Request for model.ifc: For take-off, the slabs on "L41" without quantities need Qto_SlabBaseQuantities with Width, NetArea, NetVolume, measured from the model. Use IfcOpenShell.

First a look at what the model holds.

```python
import ifcopenshell
import ifcopenshell.util.element
import ifcopenshell.util.unit

model = ifcopenshell.open("model.ifc")
print(model.schema)
for unit_type in ("LENGTHUNIT", "AREAUNIT", "VOLUMEUNIT"):
    print(unit_type, ifcopenshell.util.unit.calculate_unit_scale(model, unit_type))
storey = next(s for s in model.by_type("IfcBuildingStorey") if s.Name == "L41")
slabs = [e for e in ifcopenshell.util.element.get_decomposition(storey) if e.is_a("IfcSlab")]
for e in sorted(slabs, key=lambda e: e.id()):
    print(e.id(), e.is_a(), e.Name, list(ifcopenshell.util.element.get_psets(e, qtos_only=True)), sep=" | ")
```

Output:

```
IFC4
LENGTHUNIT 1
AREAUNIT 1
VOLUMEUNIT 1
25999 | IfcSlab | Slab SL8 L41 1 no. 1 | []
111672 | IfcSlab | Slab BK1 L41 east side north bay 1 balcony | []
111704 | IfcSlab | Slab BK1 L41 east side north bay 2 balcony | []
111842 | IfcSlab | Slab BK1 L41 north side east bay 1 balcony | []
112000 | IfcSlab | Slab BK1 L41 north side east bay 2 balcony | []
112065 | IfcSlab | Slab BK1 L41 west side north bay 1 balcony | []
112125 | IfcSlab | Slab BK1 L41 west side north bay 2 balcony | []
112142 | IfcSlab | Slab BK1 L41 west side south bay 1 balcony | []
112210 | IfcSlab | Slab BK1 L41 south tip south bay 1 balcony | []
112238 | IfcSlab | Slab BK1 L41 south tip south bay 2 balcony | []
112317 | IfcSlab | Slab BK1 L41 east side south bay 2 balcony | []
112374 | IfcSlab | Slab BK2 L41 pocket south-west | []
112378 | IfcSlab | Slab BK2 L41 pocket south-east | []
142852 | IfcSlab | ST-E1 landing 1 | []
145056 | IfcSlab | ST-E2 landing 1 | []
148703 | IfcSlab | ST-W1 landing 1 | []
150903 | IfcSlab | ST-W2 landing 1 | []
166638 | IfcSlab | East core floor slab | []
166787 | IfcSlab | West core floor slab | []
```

```python
import ifcopenshell
import ifcopenshell.api.pset
import ifcopenshell.geom
import ifcopenshell.util.element
import ifcopenshell.util.shape
import ifcopenshell.util.unit

model = ifcopenshell.open("model.ifc")
unit_scale = ifcopenshell.util.unit.calculate_unit_scale(model)
area_scale = ifcopenshell.util.unit.calculate_unit_scale(model, "AREAUNIT")
volume_scale = ifcopenshell.util.unit.calculate_unit_scale(model, "VOLUMEUNIT")
settings = ifcopenshell.geom.settings()

storey = next(s for s in model.by_type("IfcBuildingStorey") if s.Name == "L41")
slabs = [e for e in ifcopenshell.util.element.get_decomposition(storey) if e.is_a("IfcSlab")]

for e in sorted(slabs, key=lambda e: e.id()):
    if ifcopenshell.util.element.get_psets(e, qtos_only=True, should_inherit=False):
        continue
    # Geometry comes back in metres, in the element's own axes.
    shape = ifcopenshell.geom.create_shape(settings, e)
    values = {
        "Width": ifcopenshell.util.shape.get_z(shape.geometry) / unit_scale,
        "NetArea": ifcopenshell.util.shape.get_footprint_area(shape.geometry) / area_scale,
        "NetVolume": ifcopenshell.util.shape.get_volume(shape.geometry) / volume_scale,
    }
    qto = ifcopenshell.api.pset.add_qto(model, product=e, name="Qto_SlabBaseQuantities")
    ifcopenshell.api.pset.edit_qto(model, qto=qto, properties=values)
    print(e.id(), {k: round(v, 3) for k, v in values.items()})

model.write("model_updated.ifc")
```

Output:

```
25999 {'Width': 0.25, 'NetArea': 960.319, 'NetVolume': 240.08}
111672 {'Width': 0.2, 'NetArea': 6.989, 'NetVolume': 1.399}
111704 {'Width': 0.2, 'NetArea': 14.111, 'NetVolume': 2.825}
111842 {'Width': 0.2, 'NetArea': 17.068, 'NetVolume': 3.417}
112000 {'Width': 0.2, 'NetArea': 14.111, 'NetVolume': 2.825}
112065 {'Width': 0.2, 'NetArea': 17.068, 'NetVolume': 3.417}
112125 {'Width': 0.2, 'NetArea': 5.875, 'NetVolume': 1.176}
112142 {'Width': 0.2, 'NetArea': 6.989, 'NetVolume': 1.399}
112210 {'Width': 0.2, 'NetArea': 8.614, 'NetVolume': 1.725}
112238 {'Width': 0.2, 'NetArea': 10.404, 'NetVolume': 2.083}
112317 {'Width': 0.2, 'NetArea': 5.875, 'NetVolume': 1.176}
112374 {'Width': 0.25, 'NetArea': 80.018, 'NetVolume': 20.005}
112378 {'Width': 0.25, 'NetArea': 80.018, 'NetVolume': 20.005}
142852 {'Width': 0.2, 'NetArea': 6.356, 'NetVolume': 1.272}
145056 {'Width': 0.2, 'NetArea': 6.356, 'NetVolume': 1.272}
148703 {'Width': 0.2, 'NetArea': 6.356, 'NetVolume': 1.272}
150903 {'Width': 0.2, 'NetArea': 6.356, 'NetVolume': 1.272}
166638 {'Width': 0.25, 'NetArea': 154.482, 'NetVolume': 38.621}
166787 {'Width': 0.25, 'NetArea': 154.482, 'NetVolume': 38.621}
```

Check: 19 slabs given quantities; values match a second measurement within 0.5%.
